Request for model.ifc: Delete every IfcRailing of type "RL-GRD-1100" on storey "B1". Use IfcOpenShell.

First a look at what the model holds.

```python
import ifcopenshell
import ifcopenshell.util.element

model = ifcopenshell.open("model.ifc")
print(model.schema)
storey = next(s for s in model.by_type("IfcBuildingStorey") if s.Name == "B1")
railings = [e for e in ifcopenshell.util.element.get_decomposition(storey) if e.is_a("IfcRailing")]
seen = {}
for e in railings:
    element_type = ifcopenshell.util.element.get_type(e)
    name = element_type.Name if element_type not in (None, e) else None
    seen[name] = seen.get(name, 0) + 1
for name, count in sorted(seen.items(), key=str):
    print(count, "x", name)
```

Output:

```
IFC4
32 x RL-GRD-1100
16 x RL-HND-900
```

```python
import ifcopenshell
import ifcopenshell.api.root
import ifcopenshell.util.element

model = ifcopenshell.open("model.ifc")

storey = next(s for s in model.by_type("IfcBuildingStorey") if s.Name == "B1")
railings = [e for e in ifcopenshell.util.element.get_decomposition(storey) if e.is_a("IfcRailing")]
targets = [e for e in railings if (t := ifcopenshell.util.element.get_type(e)) not in (None, e) and t.Name == "RL-GRD-1100"]

for e in targets:
    ifcopenshell.api.root.remove_product(model, product=e)
print(len(targets), "removed")

model.write("model_updated.ifc")
```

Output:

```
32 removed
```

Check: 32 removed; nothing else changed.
